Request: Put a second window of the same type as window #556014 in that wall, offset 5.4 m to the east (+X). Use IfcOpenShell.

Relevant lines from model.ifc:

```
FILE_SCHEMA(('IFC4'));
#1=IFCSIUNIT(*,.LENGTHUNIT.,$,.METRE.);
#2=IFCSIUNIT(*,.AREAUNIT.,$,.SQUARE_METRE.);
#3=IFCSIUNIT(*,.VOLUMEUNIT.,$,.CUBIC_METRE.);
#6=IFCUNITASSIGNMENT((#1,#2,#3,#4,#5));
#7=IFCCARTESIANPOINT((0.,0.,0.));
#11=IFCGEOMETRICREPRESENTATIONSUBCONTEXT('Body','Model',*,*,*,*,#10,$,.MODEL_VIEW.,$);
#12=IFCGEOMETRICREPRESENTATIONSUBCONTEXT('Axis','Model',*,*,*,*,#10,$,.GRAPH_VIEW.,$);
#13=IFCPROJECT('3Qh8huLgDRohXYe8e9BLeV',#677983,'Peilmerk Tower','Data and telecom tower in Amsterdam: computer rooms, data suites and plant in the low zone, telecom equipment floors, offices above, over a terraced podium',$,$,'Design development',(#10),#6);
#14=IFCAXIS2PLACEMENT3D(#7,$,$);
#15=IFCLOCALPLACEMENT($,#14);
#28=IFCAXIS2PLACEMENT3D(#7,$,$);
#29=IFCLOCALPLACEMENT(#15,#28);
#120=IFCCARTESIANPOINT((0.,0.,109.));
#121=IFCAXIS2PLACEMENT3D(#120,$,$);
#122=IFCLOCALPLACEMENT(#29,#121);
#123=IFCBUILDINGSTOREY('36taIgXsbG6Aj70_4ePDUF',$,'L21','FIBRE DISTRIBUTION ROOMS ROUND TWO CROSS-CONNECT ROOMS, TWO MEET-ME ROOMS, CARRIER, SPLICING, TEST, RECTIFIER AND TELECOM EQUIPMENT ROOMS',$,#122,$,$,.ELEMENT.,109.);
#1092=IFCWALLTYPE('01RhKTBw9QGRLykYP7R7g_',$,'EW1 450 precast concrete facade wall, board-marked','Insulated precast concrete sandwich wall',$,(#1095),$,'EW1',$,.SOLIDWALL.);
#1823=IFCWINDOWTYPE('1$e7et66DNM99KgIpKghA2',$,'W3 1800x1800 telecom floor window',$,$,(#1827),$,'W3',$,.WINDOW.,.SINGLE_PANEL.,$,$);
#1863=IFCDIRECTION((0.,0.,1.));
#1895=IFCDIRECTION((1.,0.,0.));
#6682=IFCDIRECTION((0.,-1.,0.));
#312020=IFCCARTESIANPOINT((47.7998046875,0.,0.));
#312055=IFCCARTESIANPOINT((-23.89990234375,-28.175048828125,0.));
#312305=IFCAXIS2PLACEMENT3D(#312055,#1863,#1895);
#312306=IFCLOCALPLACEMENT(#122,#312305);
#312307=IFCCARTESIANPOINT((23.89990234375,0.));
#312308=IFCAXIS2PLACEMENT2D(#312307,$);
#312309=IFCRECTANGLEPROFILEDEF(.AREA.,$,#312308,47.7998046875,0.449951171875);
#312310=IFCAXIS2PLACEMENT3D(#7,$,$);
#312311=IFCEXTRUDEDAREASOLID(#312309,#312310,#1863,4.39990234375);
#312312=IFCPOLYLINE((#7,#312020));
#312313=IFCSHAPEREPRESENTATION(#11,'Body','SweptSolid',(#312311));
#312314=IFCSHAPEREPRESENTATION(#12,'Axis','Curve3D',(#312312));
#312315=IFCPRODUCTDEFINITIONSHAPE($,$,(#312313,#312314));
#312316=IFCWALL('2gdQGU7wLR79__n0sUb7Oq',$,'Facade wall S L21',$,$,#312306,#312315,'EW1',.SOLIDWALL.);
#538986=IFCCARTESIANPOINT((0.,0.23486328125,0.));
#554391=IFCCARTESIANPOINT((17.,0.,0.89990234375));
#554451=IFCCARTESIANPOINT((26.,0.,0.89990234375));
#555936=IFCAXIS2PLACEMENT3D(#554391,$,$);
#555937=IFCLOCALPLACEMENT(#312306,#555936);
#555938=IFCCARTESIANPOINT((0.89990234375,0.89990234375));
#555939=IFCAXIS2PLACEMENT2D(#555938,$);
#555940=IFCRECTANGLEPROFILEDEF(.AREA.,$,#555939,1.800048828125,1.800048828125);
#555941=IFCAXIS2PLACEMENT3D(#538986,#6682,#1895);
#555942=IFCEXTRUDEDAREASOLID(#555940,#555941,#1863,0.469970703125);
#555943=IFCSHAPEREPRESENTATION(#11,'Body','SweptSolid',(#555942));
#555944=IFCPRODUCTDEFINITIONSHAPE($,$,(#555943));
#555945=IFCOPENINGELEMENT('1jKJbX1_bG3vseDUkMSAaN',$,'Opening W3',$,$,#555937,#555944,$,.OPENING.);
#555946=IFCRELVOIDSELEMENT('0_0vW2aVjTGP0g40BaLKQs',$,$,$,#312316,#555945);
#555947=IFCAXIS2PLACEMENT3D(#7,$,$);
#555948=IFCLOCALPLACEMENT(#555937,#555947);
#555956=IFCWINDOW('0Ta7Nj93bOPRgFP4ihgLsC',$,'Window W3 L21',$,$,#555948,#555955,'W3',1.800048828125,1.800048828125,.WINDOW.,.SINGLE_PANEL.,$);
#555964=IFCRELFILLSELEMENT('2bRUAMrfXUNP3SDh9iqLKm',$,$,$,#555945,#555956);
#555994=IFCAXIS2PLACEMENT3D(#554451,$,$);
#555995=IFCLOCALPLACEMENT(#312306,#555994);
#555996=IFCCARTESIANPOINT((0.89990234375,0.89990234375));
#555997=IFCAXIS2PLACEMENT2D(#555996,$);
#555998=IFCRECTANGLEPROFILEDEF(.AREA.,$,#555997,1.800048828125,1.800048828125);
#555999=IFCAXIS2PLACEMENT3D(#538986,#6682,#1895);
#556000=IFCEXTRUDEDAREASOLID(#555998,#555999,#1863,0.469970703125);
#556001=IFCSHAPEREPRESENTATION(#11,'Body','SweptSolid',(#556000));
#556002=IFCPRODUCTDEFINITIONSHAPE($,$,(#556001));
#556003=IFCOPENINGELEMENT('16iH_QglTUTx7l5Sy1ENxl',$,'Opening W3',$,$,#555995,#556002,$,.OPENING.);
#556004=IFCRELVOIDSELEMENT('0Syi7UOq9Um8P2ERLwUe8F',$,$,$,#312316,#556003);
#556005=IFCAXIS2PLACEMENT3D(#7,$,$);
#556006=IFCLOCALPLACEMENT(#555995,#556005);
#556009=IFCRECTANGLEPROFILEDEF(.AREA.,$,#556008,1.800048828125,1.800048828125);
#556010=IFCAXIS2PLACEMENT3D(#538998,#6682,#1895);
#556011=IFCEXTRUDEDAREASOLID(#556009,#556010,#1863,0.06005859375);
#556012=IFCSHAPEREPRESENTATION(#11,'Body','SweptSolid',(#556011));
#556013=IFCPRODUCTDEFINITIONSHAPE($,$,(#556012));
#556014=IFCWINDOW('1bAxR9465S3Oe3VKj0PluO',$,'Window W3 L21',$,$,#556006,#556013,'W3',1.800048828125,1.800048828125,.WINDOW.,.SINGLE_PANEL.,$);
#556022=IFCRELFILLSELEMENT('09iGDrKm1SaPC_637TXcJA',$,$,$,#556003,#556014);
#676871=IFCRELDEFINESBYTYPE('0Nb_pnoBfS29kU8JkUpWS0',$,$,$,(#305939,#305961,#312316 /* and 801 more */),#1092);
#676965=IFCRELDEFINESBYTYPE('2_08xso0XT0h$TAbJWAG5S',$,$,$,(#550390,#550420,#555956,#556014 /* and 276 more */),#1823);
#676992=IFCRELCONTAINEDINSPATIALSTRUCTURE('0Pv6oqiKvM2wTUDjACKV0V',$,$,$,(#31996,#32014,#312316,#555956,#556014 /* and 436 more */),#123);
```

```python
import ifcopenshell
import ifcopenshell.api.feature
import ifcopenshell.api.geometry
import ifcopenshell.api.root
import ifcopenshell.geom
import ifcopenshell.util.element
import ifcopenshell.util.placement
import ifcopenshell.util.shape

model = ifcopenshell.open("model.ifc")
settings = ifcopenshell.geom.settings()


def volume(element):
    """Net volume in cubic metres, openings subtracted."""
    shape = ifcopenshell.geom.create_shape(settings, element)
    return ifcopenshell.util.shape.get_volume(shape.geometry)


window = model.by_guid("1bAxR9465S3Oe3VKj0PluO")
opening = window.FillsVoids[0].RelatingOpeningElement
wall = opening.VoidsElements[0].RelatingBuildingElement
before = volume(wall)
shift = ifcopenshell.util.placement.get_local_placement(wall.ObjectPlacement)[:3, 0] * 5.4

# copy_class copies the void relationship, type, container and properties, but no geometry.
new_opening = ifcopenshell.api.root.copy_class(model, product=opening)
new_opening.Representation = ifcopenshell.util.element.copy_deep(
    model, opening.Representation, exclude=["IfcGeometricRepresentationContext", "IfcRepresentationMap"]
)
new_window = ifcopenshell.api.root.copy_class(model, product=window)
new_window.Representation = ifcopenshell.util.element.copy_deep(
    model, window.Representation, exclude=["IfcGeometricRepresentationContext", "IfcRepresentationMap"]
)
new_window.Tag = None
ifcopenshell.api.feature.add_filling(model, opening=new_opening, element=new_window)

for old, new in ((opening, new_opening), (window, new_window)):
    matrix = ifcopenshell.util.placement.get_local_placement(old.ObjectPlacement)
    matrix[:3, 3] += shift
    ifcopenshell.api.geometry.edit_object_placement(model, product=new, matrix=matrix, is_si=False)

after = volume(wall)

print(f"wall volume {before:.3f} -> {after:.3f} m3")

model.write("model-out.ifc")
```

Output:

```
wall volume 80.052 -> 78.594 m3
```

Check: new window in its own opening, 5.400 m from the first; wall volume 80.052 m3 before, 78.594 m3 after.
